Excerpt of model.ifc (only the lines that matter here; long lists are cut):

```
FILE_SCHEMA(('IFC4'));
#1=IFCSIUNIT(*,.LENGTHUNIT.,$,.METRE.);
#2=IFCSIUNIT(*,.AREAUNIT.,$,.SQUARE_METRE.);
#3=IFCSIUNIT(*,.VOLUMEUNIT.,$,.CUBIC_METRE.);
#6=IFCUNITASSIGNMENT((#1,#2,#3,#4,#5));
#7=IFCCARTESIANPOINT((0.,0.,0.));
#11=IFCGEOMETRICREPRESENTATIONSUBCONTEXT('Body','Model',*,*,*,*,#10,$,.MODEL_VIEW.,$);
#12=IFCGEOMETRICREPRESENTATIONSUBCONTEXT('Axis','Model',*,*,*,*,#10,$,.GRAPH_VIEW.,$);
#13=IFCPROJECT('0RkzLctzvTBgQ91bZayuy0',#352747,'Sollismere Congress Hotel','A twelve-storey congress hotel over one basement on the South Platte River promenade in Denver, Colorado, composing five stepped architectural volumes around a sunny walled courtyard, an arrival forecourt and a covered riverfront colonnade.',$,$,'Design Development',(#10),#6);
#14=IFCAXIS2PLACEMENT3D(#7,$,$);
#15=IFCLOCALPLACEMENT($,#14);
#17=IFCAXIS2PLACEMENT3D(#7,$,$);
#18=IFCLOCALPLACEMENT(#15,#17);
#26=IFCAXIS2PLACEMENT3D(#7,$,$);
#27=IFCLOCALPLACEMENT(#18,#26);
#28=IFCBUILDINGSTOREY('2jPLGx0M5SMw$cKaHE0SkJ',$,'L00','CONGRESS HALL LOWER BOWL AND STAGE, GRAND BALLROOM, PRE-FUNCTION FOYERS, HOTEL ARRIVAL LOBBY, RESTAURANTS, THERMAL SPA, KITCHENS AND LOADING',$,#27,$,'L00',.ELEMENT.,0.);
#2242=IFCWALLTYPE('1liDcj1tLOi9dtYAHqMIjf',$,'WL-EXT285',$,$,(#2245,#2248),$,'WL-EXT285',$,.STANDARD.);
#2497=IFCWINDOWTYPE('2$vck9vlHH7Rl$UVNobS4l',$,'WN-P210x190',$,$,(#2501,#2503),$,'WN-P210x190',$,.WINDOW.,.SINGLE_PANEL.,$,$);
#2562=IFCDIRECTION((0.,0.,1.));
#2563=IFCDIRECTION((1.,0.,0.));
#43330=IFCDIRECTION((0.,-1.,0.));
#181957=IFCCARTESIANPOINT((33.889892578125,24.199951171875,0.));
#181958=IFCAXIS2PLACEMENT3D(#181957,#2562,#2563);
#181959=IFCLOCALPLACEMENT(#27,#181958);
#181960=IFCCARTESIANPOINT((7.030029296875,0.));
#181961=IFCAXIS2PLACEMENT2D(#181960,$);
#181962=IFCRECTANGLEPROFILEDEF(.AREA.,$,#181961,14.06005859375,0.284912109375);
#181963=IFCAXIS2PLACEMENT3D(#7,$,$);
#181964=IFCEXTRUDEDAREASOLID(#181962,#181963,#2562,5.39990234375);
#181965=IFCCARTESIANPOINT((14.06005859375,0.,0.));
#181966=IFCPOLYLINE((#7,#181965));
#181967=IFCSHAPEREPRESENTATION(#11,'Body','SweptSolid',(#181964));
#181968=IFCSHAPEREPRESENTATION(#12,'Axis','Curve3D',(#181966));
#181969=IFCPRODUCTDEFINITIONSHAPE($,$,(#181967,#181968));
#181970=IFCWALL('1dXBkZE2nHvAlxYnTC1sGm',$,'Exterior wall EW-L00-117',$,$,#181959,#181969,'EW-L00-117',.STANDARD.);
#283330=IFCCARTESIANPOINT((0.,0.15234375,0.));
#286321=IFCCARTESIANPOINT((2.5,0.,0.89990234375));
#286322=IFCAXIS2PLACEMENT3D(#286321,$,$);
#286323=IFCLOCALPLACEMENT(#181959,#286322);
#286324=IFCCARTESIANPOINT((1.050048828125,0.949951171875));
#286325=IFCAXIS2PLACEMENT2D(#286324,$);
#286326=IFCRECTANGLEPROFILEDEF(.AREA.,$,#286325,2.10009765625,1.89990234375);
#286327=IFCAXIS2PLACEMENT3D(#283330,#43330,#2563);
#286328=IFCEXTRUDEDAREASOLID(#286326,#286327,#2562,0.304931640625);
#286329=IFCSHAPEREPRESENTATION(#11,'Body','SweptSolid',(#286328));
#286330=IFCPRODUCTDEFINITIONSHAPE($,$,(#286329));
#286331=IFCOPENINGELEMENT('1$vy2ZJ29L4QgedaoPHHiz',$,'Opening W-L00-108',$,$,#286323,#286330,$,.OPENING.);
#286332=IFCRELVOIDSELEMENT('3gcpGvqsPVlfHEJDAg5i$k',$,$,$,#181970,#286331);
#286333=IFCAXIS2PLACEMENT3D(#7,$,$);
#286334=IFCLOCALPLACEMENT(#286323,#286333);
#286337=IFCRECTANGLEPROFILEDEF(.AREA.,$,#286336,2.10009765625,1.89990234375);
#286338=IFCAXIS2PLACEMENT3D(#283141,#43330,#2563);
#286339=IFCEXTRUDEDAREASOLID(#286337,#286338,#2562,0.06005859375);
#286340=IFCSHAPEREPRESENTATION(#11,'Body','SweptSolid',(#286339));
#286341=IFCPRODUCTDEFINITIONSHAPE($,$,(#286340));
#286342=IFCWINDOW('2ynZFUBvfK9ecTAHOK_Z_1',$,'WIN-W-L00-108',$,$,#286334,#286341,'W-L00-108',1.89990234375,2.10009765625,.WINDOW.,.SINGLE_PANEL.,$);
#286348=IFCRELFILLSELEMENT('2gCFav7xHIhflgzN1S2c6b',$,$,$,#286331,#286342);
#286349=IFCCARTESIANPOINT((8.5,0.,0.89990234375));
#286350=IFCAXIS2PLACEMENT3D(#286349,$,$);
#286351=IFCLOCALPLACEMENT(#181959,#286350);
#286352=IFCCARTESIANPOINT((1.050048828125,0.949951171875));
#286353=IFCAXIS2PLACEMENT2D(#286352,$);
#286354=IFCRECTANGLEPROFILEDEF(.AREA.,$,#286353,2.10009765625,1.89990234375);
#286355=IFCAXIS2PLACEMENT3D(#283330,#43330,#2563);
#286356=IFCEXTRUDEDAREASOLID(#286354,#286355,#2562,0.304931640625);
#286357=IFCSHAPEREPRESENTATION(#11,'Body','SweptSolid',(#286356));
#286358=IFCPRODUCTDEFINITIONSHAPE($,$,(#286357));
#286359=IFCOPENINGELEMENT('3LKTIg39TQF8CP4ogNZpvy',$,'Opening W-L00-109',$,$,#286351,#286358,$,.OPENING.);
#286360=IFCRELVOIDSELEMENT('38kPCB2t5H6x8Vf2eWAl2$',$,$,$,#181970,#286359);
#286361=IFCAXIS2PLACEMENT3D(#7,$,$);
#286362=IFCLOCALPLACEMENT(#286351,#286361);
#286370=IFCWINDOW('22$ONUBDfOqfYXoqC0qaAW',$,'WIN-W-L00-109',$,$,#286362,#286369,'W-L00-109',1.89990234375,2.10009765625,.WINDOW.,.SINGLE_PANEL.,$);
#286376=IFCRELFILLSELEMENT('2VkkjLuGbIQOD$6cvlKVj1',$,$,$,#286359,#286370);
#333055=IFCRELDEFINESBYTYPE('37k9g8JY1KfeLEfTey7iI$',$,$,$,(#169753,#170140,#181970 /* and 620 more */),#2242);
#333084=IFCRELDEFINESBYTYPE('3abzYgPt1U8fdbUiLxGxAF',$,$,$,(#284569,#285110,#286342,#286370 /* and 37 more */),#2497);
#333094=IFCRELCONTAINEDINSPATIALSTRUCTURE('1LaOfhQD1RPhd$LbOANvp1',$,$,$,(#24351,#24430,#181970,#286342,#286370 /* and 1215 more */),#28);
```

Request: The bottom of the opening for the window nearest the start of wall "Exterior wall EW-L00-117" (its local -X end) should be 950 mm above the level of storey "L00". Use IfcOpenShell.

```python
import numpy as np
import ifcopenshell
import ifcopenshell.api.geometry
import ifcopenshell.geom
import ifcopenshell.util.element
import ifcopenshell.util.placement
import ifcopenshell.util.shape
import ifcopenshell.util.unit

model = ifcopenshell.open("model.ifc")
unit_scale = ifcopenshell.util.unit.calculate_unit_scale(model)

window = model.by_guid("2ynZFUBvfK9ecTAHOK_Z_1")
opening = window.FillsVoids[0].RelatingOpeningElement
storey = ifcopenshell.util.element.get_container(window, ifc_class="IfcBuildingStorey")
level = ifcopenshell.util.placement.get_local_placement(storey.ObjectPlacement)[2, 3]

# The opening's origin need not be at the sill, so measure its lowest point.
shape = ifcopenshell.geom.create_shape(ifcopenshell.geom.settings(), opening)
bottom = ifcopenshell.util.shape.get_shape_bottom_elevation(shape, shape.geometry) / unit_scale
dz = level + 0.95 / unit_scale - bottom

shift = np.array([0.0, 0.0, dz])
# The window is placed relative to its opening, so it follows when the opening moves.
matrix = ifcopenshell.util.placement.get_local_placement(opening.ObjectPlacement)
matrix[:3, 3] += shift
ifcopenshell.api.geometry.edit_object_placement(
    model, product=opening, matrix=matrix, is_si=False, should_transform_children=True
)

print(f"moved by {dz * unit_scale:+.3f} m")

model.write("model_updated.ifc")
```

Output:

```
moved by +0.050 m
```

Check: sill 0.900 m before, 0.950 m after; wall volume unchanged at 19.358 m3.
